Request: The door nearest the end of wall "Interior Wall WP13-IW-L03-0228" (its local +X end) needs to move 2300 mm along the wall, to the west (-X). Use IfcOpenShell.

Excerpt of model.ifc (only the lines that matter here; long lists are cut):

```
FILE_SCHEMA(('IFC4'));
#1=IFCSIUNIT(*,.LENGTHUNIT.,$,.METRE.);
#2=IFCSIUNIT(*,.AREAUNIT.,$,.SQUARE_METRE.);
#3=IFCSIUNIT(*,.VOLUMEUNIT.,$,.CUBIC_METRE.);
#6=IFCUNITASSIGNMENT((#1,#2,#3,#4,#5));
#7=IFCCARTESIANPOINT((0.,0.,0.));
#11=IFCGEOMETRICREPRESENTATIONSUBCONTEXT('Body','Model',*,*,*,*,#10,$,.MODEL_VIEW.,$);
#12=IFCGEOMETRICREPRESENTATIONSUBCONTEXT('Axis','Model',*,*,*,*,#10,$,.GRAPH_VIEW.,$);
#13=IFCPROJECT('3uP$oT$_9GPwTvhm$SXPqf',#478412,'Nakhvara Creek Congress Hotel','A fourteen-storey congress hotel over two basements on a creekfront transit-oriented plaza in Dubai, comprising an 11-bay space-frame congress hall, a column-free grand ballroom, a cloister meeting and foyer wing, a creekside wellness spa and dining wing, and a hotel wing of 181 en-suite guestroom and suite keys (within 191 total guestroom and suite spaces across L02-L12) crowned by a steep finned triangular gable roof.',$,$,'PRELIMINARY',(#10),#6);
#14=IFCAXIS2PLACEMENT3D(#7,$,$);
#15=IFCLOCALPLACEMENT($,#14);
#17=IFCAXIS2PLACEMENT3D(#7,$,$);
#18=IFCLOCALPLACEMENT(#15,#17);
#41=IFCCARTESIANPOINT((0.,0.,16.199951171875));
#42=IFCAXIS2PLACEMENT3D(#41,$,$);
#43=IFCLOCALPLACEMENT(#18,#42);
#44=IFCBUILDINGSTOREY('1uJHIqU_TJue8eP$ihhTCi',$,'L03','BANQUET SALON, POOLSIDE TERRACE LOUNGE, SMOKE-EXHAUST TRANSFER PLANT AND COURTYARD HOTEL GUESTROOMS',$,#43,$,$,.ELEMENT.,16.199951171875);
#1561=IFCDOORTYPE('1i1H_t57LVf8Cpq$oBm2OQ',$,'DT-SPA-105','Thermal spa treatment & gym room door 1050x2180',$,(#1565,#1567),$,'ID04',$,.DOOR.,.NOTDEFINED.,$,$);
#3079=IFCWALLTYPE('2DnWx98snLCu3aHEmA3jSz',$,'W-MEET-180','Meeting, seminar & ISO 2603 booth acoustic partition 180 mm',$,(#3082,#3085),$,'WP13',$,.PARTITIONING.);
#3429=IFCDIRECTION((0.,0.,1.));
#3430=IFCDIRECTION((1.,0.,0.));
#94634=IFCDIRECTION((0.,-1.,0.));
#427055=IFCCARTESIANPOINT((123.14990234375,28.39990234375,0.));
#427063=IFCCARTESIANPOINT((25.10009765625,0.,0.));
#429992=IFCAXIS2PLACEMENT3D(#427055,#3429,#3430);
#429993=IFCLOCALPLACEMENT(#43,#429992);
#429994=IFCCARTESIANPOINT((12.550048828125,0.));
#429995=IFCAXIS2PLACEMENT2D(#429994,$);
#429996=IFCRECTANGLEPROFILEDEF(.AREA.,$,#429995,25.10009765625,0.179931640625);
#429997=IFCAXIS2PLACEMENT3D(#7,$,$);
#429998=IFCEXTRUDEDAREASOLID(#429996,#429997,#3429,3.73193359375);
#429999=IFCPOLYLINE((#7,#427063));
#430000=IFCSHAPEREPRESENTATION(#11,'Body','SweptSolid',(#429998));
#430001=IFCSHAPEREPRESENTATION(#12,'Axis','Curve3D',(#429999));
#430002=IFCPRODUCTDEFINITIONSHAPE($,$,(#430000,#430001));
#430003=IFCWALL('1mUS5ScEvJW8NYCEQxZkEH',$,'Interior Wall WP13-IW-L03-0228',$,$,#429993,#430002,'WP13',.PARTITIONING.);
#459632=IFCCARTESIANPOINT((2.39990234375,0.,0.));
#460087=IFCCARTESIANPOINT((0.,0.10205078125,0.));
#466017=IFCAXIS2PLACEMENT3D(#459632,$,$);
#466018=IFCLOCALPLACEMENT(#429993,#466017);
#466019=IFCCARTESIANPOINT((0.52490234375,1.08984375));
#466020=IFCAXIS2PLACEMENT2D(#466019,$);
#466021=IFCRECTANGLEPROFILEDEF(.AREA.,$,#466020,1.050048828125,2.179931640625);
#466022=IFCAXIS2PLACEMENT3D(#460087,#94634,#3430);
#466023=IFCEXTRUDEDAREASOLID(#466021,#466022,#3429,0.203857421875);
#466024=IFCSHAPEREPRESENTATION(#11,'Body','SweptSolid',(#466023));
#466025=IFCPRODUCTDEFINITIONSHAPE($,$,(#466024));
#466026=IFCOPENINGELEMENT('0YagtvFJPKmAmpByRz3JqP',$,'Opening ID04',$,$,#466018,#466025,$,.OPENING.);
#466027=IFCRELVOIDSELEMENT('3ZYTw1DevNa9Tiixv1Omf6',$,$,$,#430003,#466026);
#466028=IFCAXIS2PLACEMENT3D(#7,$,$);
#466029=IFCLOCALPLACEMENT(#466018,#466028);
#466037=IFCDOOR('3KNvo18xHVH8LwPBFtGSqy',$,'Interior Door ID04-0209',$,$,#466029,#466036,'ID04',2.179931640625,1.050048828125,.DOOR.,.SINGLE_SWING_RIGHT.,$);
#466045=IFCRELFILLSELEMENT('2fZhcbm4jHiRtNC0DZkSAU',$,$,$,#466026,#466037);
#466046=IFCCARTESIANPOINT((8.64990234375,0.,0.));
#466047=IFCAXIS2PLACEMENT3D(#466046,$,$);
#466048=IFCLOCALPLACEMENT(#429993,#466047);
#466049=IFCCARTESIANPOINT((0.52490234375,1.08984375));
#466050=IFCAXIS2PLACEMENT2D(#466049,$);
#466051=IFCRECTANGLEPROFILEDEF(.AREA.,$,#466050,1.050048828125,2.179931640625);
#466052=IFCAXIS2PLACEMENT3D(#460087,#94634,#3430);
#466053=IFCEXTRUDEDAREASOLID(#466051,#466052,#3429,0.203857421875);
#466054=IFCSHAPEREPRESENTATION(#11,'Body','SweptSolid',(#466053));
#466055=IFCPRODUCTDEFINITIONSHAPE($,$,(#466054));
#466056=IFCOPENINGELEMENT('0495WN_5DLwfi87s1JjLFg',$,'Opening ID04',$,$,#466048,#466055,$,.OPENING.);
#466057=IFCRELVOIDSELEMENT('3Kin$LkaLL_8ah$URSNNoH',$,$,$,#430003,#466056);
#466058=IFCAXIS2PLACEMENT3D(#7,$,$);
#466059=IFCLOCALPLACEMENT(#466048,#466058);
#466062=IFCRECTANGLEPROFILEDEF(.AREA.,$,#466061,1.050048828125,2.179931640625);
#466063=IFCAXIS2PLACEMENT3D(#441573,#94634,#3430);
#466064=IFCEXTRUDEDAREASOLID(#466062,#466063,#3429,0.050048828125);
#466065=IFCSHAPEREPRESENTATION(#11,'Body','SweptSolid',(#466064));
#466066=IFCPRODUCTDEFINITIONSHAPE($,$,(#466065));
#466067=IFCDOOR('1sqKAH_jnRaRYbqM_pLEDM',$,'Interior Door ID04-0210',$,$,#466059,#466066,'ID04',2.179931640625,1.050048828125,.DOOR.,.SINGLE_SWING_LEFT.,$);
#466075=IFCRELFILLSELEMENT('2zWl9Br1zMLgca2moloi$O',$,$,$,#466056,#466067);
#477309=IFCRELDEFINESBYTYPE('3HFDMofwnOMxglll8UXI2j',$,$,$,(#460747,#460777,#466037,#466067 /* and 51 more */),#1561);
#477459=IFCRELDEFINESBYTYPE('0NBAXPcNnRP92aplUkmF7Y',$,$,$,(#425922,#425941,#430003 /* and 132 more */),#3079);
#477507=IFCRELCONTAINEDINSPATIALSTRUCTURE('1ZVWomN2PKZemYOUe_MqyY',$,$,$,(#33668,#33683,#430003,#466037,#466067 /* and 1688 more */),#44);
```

```python
import ifcopenshell
import ifcopenshell.api.geometry
import ifcopenshell.util.placement
import ifcopenshell.util.unit

model = ifcopenshell.open("model.ifc")
unit_scale = ifcopenshell.util.unit.calculate_unit_scale(model)

door = model.by_id(466067)
opening = door.FillsVoids[0].RelatingOpeningElement
wall = opening.VoidsElements[0].RelatingBuildingElement

wall_matrix = ifcopenshell.util.placement.get_local_placement(wall.ObjectPlacement)
shift = wall_matrix[:3, 0] * -2.3 / unit_scale
before = ifcopenshell.util.placement.get_local_placement(door.ObjectPlacement)[:3, 3].copy()

# The door is placed relative to its opening, so it follows when the opening moves.
matrix = ifcopenshell.util.placement.get_local_placement(opening.ObjectPlacement)
matrix[:3, 3] += shift
ifcopenshell.api.geometry.edit_object_placement(
    model, product=opening, matrix=matrix, is_si=False, should_transform_children=True
)

after = ifcopenshell.util.placement.get_local_placement(door.ObjectPlacement)[:3, 3]
print("door moved by", (after - before).round(3) + 0.0)

model.write("model_updated.ifc")
```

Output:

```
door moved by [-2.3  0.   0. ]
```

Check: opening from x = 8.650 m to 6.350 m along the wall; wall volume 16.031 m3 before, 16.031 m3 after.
